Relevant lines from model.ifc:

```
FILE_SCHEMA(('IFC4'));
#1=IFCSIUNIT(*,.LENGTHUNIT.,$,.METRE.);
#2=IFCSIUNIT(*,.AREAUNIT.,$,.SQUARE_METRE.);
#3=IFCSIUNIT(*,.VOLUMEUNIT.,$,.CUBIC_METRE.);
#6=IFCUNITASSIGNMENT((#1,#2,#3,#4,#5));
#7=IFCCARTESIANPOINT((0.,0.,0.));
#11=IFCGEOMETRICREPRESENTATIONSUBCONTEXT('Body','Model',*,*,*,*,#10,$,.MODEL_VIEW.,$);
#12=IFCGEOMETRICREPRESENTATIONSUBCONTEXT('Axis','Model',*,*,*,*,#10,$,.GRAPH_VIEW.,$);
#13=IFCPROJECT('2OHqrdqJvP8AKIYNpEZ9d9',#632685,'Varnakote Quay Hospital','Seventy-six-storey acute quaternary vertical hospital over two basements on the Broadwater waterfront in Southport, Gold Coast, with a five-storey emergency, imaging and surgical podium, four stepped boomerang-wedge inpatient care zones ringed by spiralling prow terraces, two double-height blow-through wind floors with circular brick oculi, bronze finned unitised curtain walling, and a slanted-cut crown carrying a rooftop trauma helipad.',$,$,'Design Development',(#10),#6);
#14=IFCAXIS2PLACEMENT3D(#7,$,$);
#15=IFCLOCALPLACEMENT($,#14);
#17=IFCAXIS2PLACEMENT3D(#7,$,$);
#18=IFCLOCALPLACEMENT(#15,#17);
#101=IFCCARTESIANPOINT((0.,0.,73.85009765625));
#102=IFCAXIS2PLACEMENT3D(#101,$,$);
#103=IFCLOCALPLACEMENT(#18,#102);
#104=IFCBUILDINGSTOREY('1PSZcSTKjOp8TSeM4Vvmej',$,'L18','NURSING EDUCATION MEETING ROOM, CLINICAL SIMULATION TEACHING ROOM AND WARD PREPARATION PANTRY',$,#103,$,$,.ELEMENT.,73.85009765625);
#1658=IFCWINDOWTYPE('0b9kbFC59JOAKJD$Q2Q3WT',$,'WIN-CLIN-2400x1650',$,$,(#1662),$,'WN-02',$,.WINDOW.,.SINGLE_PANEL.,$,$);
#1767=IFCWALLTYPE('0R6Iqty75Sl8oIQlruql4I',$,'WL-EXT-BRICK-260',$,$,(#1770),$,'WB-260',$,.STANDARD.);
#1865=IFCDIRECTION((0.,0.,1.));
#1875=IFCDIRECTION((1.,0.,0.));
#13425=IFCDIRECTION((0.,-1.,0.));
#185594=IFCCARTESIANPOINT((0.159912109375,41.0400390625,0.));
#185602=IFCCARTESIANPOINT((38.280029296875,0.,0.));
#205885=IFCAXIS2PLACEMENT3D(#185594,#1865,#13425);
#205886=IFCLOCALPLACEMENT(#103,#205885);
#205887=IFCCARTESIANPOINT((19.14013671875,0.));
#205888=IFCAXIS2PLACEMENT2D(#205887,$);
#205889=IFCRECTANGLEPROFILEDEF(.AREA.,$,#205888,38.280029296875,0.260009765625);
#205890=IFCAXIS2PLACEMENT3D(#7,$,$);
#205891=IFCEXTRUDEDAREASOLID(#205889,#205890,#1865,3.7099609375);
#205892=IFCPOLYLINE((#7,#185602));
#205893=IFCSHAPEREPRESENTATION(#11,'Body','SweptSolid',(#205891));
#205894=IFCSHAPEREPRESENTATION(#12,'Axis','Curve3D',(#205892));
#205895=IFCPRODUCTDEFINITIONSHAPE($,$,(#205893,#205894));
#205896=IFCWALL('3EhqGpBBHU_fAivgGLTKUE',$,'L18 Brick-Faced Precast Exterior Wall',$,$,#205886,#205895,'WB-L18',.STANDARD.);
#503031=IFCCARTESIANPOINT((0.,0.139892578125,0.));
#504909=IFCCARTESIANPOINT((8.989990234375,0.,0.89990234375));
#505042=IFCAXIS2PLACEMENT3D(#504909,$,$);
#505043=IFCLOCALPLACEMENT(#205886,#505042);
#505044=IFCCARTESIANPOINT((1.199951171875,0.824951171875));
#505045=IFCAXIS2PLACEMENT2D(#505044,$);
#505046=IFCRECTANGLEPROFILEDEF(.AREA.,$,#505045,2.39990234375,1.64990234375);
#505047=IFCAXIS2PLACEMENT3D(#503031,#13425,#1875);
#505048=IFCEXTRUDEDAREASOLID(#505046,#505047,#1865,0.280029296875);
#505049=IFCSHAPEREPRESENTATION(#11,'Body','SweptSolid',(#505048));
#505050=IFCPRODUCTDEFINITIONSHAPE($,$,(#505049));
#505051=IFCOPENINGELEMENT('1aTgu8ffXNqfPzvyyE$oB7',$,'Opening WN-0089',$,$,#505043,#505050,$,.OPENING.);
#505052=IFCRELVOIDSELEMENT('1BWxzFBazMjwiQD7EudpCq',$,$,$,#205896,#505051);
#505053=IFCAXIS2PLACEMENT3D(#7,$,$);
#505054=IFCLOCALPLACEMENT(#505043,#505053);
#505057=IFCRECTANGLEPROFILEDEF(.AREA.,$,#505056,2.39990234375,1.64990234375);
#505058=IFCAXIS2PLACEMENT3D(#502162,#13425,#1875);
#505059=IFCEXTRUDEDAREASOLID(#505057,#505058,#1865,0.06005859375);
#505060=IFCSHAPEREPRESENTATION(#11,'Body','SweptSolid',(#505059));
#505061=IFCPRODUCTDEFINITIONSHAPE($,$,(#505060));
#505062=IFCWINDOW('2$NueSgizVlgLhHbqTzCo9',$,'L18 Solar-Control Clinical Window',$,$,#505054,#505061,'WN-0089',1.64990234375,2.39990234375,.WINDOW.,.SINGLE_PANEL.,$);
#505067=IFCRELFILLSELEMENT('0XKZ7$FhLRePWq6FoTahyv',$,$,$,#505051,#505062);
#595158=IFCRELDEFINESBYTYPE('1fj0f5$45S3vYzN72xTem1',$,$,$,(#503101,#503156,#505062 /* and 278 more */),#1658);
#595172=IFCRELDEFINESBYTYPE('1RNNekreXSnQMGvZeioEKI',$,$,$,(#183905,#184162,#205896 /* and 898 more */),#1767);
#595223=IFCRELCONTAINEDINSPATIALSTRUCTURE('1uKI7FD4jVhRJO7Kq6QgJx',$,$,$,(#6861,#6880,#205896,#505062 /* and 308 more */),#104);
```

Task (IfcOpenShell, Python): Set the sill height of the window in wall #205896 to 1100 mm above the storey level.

```python
import numpy as np
import ifcopenshell
import ifcopenshell.api.geometry
import ifcopenshell.geom
import ifcopenshell.util.element
import ifcopenshell.util.placement
import ifcopenshell.util.shape
import ifcopenshell.util.unit

model = ifcopenshell.open("model.ifc")
unit_scale = ifcopenshell.util.unit.calculate_unit_scale(model)

window = model.by_guid("2$NueSgizVlgLhHbqTzCo9")
opening = window.FillsVoids[0].RelatingOpeningElement
storey = ifcopenshell.util.element.get_container(window, ifc_class="IfcBuildingStorey")
level = ifcopenshell.util.placement.get_local_placement(storey.ObjectPlacement)[2, 3]

# The opening's origin need not be at the sill, so measure its lowest point.
shape = ifcopenshell.geom.create_shape(ifcopenshell.geom.settings(), opening)
bottom = ifcopenshell.util.shape.get_shape_bottom_elevation(shape, shape.geometry) / unit_scale
dz = level + 1.1 / unit_scale - bottom

shift = np.array([0.0, 0.0, dz])
# The window is placed relative to its opening, so it follows when the opening moves.
matrix = ifcopenshell.util.placement.get_local_placement(opening.ObjectPlacement)
matrix[:3, 3] += shift
ifcopenshell.api.geometry.edit_object_placement(
    model, product=opening, matrix=matrix, is_si=False, should_transform_children=True
)

print(f"moved by {dz * unit_scale:+.3f} m")

model.write("model-out.ifc")
```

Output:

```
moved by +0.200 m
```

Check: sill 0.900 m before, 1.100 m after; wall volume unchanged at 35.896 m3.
